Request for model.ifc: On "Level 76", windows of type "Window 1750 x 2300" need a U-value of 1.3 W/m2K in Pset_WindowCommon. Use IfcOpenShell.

First a look at what the model holds.

```python
import ifcopenshell
import ifcopenshell.util.element

model = ifcopenshell.open("model.ifc")
print(model.schema)
storey = next(s for s in model.by_type("IfcBuildingStorey") if s.Name == "Level 76")
windows = [e for e in ifcopenshell.util.element.get_decomposition(storey) if e.is_a("IfcWindow")]
seen = {}
for e in windows:
    element_type = ifcopenshell.util.element.get_type(e)
    key = (element_type.Name if element_type != e and element_type else None, ifcopenshell.util.element.get_pset(e, "Pset_WindowCommon", "ThermalTransmittance"))
    seen[key] = seen.get(key, 0) + 1
for (name, value), count in sorted(seen.items(), key=str):
    print(count, "x", name, "|", value)
```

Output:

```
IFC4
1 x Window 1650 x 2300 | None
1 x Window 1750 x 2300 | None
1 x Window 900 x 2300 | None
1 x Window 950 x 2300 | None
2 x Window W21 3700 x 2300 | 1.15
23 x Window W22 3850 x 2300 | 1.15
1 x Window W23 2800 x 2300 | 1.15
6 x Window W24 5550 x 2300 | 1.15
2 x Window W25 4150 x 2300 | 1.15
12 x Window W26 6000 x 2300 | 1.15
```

```python
import ifcopenshell
import ifcopenshell.api.pset
import ifcopenshell.util.element

model = ifcopenshell.open("model.ifc")

storey = next(s for s in model.by_type("IfcBuildingStorey") if s.Name == "Level 76")
windows = [e for e in ifcopenshell.util.element.get_decomposition(storey) if e.is_a("IfcWindow")]

count = 0
for e in windows:
    element_type = ifcopenshell.util.element.get_type(e)
    if element_type in (None, e) or element_type.Name != "Window 1750 x 2300":
        continue
    found = ifcopenshell.util.element.get_pset(e, "Pset_WindowCommon", should_inherit=False)
    if found:
        pset = model.by_id(found["id"])
        if len(ifcopenshell.util.element.get_elements_by_pset(pset)) > 1:
            pset = ifcopenshell.api.pset.unshare_pset(model, products=[e], pset=pset)[0]
    else:
        pset = ifcopenshell.api.pset.add_pset(model, product=e, name="Pset_WindowCommon")
    ifcopenshell.api.pset.edit_pset(model, pset=pset, properties={"ThermalTransmittance": 1.3})
    count += 1

print(count, "windows updated")

model.write("model_edited.ifc")
```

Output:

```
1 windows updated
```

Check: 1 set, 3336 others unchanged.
